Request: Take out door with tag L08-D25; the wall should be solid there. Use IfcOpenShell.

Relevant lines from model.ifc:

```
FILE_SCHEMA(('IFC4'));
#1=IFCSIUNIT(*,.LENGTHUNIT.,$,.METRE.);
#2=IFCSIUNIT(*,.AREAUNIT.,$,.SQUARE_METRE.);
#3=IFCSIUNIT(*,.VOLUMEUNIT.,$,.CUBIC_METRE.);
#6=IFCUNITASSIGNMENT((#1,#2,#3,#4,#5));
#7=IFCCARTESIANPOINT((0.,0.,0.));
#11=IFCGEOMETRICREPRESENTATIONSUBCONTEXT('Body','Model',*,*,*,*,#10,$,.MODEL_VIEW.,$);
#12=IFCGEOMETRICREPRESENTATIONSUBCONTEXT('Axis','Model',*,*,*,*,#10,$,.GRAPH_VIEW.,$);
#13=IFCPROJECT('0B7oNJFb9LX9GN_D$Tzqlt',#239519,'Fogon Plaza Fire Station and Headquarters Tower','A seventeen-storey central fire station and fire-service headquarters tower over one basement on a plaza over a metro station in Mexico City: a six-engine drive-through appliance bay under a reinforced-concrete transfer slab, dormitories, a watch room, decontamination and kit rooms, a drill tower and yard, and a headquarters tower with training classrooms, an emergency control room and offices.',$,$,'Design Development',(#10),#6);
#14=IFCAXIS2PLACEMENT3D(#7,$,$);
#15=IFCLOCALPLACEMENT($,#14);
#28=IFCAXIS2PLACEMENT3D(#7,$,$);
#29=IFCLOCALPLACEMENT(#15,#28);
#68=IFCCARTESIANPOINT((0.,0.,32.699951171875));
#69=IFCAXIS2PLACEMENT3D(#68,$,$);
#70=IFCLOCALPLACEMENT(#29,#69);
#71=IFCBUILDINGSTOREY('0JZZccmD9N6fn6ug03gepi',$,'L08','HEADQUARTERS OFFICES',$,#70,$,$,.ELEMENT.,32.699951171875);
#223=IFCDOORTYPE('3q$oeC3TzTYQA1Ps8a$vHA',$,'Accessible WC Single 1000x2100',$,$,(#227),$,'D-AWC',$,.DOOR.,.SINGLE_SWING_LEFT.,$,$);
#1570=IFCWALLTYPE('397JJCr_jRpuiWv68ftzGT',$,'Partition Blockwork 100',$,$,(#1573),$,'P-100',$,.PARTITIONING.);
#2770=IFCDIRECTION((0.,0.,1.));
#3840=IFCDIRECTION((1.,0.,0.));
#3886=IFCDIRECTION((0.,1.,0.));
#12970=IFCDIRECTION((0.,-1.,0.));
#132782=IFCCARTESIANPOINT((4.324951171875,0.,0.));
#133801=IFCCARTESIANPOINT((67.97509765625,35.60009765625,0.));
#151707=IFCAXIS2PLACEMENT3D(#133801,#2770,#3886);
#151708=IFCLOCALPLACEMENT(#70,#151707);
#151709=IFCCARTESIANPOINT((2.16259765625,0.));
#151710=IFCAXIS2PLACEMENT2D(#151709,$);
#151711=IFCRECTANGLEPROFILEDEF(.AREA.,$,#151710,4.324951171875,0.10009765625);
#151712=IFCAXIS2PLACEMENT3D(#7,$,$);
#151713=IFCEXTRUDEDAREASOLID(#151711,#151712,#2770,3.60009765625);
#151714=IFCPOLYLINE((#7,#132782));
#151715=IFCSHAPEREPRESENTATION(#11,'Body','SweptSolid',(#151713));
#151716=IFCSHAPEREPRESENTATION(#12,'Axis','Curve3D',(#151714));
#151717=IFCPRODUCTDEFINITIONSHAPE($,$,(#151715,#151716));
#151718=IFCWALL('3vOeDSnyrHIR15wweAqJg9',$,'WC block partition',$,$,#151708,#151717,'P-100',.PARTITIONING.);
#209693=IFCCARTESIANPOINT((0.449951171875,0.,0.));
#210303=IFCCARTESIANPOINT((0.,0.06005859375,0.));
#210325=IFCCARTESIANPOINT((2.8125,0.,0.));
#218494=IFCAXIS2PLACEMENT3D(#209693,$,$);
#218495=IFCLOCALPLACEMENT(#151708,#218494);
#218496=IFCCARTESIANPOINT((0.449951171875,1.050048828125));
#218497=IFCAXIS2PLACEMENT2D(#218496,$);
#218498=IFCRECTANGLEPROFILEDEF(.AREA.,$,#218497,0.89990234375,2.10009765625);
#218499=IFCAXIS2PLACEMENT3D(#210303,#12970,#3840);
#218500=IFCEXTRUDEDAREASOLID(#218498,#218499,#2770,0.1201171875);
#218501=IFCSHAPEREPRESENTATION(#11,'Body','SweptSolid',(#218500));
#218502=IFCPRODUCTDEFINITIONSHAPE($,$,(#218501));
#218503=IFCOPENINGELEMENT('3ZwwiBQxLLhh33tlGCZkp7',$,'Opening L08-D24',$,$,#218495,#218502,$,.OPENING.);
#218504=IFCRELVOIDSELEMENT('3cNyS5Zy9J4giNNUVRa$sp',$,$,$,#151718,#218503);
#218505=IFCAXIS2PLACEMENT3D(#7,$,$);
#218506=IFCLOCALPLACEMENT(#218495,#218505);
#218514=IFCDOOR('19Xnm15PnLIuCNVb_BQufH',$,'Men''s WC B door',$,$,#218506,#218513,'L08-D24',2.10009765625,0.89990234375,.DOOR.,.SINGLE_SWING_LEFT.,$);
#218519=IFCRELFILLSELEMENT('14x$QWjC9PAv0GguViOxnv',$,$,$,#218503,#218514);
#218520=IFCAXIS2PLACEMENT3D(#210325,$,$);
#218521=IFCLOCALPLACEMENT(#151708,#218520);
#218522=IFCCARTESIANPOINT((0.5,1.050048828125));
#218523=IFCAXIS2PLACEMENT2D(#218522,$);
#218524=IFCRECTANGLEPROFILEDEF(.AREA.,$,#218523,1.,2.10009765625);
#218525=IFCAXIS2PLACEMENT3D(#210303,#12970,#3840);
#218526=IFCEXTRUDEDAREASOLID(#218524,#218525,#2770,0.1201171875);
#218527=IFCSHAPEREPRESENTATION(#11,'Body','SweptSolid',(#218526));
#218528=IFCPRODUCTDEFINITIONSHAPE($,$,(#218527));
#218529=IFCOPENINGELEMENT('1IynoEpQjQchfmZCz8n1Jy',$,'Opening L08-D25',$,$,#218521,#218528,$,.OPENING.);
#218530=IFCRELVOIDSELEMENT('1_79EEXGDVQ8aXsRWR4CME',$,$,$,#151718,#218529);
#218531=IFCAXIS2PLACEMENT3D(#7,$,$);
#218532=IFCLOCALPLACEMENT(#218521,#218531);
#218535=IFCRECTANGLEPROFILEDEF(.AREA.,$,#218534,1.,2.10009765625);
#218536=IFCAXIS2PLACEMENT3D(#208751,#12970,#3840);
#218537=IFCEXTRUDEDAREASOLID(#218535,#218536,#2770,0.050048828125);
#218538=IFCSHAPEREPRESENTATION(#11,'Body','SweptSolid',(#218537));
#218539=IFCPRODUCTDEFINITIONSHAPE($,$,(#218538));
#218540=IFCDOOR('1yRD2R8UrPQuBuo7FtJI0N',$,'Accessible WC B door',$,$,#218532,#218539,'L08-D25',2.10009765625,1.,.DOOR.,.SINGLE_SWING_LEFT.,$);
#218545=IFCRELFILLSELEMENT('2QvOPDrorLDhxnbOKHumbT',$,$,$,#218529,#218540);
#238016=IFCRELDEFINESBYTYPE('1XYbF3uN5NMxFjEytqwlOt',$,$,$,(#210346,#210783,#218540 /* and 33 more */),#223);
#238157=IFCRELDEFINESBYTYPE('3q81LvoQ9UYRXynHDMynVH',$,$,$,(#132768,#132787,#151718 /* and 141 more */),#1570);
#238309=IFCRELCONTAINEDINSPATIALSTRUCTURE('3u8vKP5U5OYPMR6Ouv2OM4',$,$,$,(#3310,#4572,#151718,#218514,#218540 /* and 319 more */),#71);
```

```python
import ifcopenshell
import ifcopenshell.api.feature
import ifcopenshell.api.root
import ifcopenshell.geom
import ifcopenshell.util.shape

model = ifcopenshell.open("model.ifc")
settings = ifcopenshell.geom.settings()


def volume(element):
    """Net volume in cubic metres, openings subtracted."""
    shape = ifcopenshell.geom.create_shape(settings, element)
    return ifcopenshell.util.shape.get_volume(shape.geometry)


door = model.by_id(218540)
opening = door.FillsVoids[0].RelatingOpeningElement
wall = opening.VoidsElements[0].RelatingBuildingElement
before = volume(wall)

ifcopenshell.api.root.remove_product(model, product=door)
ifcopenshell.api.feature.remove_feature(model, feature=opening)

after = volume(wall)

print(f"wall volume {before:.3f} -> {after:.3f} m3")

model.write("model_edited.ifc")
```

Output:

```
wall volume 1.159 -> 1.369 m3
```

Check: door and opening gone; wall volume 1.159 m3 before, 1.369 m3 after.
